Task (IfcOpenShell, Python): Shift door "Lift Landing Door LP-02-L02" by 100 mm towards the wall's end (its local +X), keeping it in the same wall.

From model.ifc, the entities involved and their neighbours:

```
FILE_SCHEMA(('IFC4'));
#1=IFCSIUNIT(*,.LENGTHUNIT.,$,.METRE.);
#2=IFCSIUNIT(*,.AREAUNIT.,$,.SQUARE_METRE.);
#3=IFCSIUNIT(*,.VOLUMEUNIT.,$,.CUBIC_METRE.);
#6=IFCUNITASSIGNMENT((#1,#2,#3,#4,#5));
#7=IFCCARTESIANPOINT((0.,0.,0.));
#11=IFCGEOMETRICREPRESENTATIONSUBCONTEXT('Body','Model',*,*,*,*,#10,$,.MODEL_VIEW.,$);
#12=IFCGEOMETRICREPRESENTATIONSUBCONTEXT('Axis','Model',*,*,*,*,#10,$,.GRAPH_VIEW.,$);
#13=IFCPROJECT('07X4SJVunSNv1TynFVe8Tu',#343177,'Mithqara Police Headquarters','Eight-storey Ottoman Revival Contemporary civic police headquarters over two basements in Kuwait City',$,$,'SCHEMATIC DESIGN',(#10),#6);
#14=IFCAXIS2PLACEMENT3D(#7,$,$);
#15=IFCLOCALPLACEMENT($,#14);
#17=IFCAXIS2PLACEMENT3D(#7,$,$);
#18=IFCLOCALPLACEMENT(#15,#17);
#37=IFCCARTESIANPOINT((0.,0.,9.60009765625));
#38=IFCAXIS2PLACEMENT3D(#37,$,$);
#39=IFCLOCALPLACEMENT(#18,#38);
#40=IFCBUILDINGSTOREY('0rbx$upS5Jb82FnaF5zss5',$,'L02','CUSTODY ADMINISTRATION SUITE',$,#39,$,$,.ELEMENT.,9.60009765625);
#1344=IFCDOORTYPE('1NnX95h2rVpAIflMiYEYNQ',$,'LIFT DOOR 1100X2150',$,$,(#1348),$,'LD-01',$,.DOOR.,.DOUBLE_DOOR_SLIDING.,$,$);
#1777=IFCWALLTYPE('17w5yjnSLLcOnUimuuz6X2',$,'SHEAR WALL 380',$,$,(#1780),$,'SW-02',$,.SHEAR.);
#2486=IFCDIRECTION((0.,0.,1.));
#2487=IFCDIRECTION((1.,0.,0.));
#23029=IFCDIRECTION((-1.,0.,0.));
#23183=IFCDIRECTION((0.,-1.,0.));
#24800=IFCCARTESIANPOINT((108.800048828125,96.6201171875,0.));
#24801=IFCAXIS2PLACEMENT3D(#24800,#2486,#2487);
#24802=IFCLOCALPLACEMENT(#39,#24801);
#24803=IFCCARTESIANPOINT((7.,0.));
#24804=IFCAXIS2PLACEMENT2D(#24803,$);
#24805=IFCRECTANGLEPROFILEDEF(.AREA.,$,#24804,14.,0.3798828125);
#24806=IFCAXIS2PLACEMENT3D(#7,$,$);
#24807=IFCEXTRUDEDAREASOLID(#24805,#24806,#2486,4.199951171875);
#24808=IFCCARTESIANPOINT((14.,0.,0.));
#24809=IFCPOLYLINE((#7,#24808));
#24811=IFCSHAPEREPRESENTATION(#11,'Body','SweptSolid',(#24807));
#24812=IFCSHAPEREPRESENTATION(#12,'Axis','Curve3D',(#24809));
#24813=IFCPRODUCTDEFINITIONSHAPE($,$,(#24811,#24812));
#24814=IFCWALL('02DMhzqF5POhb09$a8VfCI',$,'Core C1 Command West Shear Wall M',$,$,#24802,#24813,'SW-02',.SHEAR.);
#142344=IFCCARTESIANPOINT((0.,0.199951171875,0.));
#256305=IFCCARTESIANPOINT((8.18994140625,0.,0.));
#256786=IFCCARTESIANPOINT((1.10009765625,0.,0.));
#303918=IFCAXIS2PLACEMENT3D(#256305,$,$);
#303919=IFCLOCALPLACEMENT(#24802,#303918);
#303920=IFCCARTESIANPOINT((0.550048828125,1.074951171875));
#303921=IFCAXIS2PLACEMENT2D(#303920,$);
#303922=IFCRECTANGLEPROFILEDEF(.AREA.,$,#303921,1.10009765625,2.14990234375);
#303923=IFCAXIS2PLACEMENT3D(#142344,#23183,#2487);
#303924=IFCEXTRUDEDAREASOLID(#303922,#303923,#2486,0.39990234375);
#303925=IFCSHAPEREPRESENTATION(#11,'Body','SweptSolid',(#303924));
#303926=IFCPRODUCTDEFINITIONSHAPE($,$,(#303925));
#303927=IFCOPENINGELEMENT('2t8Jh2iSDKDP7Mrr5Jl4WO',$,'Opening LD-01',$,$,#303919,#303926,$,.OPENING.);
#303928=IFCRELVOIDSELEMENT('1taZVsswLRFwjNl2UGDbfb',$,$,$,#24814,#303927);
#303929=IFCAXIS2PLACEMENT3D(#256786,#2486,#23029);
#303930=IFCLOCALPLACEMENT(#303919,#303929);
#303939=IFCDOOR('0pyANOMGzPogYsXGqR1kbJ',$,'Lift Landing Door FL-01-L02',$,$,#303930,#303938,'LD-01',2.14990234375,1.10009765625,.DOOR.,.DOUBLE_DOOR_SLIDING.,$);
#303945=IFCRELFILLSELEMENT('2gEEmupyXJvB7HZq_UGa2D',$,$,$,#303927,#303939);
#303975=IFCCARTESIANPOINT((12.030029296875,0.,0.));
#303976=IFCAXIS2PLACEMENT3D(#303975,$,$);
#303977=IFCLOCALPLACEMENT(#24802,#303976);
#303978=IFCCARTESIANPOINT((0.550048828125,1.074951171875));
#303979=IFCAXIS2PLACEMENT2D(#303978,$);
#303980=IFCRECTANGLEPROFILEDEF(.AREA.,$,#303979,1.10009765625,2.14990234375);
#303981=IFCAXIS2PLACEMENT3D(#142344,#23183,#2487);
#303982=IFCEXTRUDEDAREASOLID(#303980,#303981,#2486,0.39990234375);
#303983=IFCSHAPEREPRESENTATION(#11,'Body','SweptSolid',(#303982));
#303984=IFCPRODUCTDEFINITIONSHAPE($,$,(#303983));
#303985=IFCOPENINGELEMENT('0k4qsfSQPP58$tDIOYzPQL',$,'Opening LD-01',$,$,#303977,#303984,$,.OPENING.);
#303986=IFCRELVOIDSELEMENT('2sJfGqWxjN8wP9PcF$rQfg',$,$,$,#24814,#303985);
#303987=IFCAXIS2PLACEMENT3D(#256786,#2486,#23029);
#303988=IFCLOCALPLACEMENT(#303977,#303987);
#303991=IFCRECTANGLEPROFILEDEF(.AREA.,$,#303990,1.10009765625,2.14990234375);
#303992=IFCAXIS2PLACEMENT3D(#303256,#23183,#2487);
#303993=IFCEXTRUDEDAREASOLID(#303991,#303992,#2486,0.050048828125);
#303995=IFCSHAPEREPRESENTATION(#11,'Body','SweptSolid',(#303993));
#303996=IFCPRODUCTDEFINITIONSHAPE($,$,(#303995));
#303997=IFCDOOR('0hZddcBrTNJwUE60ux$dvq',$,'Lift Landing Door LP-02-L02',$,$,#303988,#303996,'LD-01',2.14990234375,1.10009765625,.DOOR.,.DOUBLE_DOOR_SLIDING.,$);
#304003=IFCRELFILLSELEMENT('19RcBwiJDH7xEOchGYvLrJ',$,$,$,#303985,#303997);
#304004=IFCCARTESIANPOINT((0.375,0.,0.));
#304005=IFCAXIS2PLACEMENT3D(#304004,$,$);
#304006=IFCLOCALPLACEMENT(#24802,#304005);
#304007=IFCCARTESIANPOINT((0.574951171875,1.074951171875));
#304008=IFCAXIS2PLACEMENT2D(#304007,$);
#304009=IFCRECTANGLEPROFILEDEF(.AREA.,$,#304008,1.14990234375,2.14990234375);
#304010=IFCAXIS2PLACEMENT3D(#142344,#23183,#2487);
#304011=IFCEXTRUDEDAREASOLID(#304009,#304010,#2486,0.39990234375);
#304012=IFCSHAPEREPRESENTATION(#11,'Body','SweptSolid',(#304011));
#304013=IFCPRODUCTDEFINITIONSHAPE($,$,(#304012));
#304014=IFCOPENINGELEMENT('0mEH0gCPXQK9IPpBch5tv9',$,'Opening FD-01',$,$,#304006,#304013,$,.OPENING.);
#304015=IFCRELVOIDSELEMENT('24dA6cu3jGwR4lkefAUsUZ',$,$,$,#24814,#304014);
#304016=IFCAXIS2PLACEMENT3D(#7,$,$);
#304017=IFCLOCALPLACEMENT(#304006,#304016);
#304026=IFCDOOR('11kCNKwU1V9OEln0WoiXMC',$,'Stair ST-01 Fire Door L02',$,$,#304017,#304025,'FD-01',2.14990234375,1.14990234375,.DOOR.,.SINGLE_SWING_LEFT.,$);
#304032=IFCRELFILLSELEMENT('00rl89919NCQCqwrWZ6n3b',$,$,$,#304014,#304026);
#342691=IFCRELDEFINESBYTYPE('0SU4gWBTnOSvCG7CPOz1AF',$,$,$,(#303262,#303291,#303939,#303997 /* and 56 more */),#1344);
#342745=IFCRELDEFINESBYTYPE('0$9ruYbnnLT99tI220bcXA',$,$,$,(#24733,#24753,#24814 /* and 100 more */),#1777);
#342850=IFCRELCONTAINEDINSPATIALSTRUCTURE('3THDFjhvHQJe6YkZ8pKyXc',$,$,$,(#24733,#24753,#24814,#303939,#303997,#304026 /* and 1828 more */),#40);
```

```python
import ifcopenshell
import ifcopenshell.api.geometry
import ifcopenshell.util.placement

model = ifcopenshell.open("model.ifc")

door = model.by_id(303997)
opening = door.FillsVoids[0].RelatingOpeningElement
wall = opening.VoidsElements[0].RelatingBuildingElement

wall_matrix = ifcopenshell.util.placement.get_local_placement(wall.ObjectPlacement)
shift = wall_matrix[:3, 0] * 0.1
before = ifcopenshell.util.placement.get_local_placement(door.ObjectPlacement)[:3, 3].copy()

# The door is placed relative to its opening, so it follows when the opening moves.
matrix = ifcopenshell.util.placement.get_local_placement(opening.ObjectPlacement)
matrix[:3, 3] += shift
ifcopenshell.api.geometry.edit_object_placement(
    model, product=opening, matrix=matrix, is_si=False, should_transform_children=True
)

after = ifcopenshell.util.placement.get_local_placement(door.ObjectPlacement)[:3, 3]
print("door moved by", (after - before).round(3) + 0.0)

model.write("model-out.ifc")
```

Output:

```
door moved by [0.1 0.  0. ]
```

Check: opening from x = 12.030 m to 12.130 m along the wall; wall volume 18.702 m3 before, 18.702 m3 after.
